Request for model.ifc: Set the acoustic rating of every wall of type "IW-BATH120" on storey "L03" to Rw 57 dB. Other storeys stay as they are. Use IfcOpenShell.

First a look at what the model holds.

```python
import ifcopenshell
import ifcopenshell.util.element

model = ifcopenshell.open("model.ifc")
print(model.schema)
storey = next(s for s in model.by_type("IfcBuildingStorey") if s.Name == "L03")
walls = [e for e in ifcopenshell.util.element.get_decomposition(storey) if e.is_a("IfcWall")]
seen = {}
for e in walls:
    element_type = ifcopenshell.util.element.get_type(e)
    key = (element_type.Name if element_type != e and element_type else None, ifcopenshell.util.element.get_pset(e, "Pset_WallCommon", "AcousticRating"))
    seen[key] = seen.get(key, 0) + 1
for (name, value), count in sorted(seen.items(), key=str):
    print(count, "x", name, "|", value)
```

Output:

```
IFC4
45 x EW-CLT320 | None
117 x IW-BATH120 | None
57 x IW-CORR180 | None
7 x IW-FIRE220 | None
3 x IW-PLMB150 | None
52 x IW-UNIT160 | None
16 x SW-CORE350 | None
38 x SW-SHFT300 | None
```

```python
import ifcopenshell
import ifcopenshell.api.pset
import ifcopenshell.util.element

model = ifcopenshell.open("model.ifc")

storey = next(s for s in model.by_type("IfcBuildingStorey") if s.Name == "L03")
walls = [e for e in ifcopenshell.util.element.get_decomposition(storey) if e.is_a("IfcWall")]

count = 0
for e in walls:
    element_type = ifcopenshell.util.element.get_type(e)
    if element_type in (None, e) or element_type.Name != "IW-BATH120":
        continue
    # add_pset returns the element's existing set when there is one.
    pset = ifcopenshell.api.pset.add_pset(model, product=e, name="Pset_WallCommon")
    ifcopenshell.api.pset.edit_pset(model, pset=pset, properties={"AcousticRating": "Rw 57 dB"})
    count += 1

print(count, "walls updated")

model.write("model_updated.ifc")
```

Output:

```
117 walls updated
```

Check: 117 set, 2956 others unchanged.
